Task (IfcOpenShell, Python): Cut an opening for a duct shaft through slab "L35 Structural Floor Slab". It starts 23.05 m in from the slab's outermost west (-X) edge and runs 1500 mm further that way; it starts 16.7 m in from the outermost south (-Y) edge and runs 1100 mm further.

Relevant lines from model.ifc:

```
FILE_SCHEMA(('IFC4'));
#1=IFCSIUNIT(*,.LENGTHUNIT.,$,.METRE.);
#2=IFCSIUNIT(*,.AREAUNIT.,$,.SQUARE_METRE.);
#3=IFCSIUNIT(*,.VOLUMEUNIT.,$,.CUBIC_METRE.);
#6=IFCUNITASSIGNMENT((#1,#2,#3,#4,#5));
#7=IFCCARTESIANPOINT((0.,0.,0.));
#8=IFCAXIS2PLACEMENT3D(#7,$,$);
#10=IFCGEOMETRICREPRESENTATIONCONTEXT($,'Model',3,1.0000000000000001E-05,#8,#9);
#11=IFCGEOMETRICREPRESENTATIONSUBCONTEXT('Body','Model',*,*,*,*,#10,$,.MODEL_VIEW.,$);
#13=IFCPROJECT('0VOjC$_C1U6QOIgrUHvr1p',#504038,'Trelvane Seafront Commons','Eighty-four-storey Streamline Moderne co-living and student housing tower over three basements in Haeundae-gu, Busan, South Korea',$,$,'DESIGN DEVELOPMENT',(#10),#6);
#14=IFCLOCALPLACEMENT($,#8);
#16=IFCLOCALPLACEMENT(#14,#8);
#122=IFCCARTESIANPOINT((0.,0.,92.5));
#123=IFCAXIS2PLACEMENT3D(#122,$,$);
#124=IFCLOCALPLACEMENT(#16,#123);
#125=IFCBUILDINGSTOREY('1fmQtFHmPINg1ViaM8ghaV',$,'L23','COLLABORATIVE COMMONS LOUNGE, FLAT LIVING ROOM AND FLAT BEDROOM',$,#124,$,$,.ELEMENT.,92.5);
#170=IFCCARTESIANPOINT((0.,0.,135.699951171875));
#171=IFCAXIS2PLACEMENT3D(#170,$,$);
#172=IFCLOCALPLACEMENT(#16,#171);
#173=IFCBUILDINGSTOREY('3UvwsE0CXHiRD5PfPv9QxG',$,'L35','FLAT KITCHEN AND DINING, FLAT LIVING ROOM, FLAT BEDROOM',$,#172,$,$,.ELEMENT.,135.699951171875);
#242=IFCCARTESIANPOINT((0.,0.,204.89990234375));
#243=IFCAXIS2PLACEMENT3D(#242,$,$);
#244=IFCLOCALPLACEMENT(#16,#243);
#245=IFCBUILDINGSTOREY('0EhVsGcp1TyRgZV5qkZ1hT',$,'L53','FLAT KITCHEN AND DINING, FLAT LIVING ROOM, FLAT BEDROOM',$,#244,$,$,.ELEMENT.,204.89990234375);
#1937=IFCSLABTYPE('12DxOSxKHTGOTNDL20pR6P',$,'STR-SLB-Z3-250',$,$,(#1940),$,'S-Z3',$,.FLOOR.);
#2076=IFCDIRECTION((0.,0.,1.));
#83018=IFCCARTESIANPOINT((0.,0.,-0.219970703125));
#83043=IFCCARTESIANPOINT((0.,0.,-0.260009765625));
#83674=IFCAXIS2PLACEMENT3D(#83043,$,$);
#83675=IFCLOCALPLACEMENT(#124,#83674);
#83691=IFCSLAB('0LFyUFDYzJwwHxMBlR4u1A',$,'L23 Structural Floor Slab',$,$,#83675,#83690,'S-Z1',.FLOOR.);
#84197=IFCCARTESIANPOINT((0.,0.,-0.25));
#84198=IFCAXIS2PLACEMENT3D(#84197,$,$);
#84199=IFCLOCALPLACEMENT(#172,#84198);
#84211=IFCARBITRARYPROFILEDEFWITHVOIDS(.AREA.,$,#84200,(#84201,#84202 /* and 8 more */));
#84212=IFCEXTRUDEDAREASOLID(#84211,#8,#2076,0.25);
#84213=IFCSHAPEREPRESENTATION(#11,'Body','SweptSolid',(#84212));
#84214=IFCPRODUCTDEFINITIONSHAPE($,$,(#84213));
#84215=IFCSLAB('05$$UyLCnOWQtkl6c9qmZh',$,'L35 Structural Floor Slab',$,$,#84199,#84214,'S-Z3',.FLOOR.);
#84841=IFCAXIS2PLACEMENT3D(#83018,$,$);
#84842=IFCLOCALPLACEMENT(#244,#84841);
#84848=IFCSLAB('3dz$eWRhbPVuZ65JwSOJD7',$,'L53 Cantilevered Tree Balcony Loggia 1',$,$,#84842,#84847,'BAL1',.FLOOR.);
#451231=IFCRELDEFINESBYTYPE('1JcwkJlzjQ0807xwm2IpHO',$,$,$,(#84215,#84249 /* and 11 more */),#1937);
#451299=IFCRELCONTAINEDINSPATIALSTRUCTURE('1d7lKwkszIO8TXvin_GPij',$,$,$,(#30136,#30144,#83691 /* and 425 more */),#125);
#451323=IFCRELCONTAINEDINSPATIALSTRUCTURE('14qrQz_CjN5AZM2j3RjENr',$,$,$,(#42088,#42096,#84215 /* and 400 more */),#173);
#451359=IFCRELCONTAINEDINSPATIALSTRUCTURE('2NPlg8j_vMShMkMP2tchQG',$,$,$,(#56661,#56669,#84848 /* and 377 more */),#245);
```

```python
import numpy as np
import ifcopenshell
import ifcopenshell.api.feature
import ifcopenshell.api.geometry
import ifcopenshell.api.root
import ifcopenshell.geom
import ifcopenshell.util.placement
import ifcopenshell.util.representation
import ifcopenshell.util.shape
import ifcopenshell.util.unit

model = ifcopenshell.open("model.ifc")
unit_scale = ifcopenshell.util.unit.calculate_unit_scale(model)
settings = ifcopenshell.geom.settings()


def volume(element):
    """Net volume in cubic metres, openings subtracted."""
    shape = ifcopenshell.geom.create_shape(settings, element)
    return ifcopenshell.util.shape.get_volume(shape.geometry)


slab = model.by_id(84215)
before = volume(slab)

# Extent in the slab's own axes, in metres. The edges named are its -X and -Y sides.
slab_shape = ifcopenshell.geom.create_shape(settings, slab)
vertices = ifcopenshell.util.shape.get_vertices(slab_shape.geometry)
x_min, y_min, bottom = vertices.min(axis=0)
top = vertices[:, 2].max()

opening = ifcopenshell.api.root.create_entity(model, ifc_class="IfcOpeningElement", name="Duct shaft opening", predefined_type="OPENING")
context = ifcopenshell.util.representation.get_context(model, "Model", "Body", "MODEL_VIEW")
width, depth = 1.5, 1.1
outline = [(0.0, 0.0), (width, 0.0), (width, depth), (0.0, depth), (0.0, 0.0)]
# Overshoot both faces by 50 mm so the cut is clean.
shape = ifcopenshell.api.geometry.add_slab_representation(
    model, context=context, depth=top - bottom + 0.1, polyline=outline
)
ifcopenshell.api.geometry.assign_representation(model, product=opening, representation=shape)

matrix = ifcopenshell.util.placement.get_local_placement(slab.ObjectPlacement)
matrix[:, 3] = matrix @ np.append(np.array([x_min + 23.05, y_min + 16.7, bottom - 0.05]) / unit_scale, 1.0)
ifcopenshell.api.geometry.edit_object_placement(model, product=opening, matrix=matrix, is_si=False)
ifcopenshell.api.feature.add_feature(model, feature=opening, element=slab)

after = volume(slab)

print(f"slab volume {before:.3f} -> {after:.3f} m3")

model.write("model_rev.ifc")
```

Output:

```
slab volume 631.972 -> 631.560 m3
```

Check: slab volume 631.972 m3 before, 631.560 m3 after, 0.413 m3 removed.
